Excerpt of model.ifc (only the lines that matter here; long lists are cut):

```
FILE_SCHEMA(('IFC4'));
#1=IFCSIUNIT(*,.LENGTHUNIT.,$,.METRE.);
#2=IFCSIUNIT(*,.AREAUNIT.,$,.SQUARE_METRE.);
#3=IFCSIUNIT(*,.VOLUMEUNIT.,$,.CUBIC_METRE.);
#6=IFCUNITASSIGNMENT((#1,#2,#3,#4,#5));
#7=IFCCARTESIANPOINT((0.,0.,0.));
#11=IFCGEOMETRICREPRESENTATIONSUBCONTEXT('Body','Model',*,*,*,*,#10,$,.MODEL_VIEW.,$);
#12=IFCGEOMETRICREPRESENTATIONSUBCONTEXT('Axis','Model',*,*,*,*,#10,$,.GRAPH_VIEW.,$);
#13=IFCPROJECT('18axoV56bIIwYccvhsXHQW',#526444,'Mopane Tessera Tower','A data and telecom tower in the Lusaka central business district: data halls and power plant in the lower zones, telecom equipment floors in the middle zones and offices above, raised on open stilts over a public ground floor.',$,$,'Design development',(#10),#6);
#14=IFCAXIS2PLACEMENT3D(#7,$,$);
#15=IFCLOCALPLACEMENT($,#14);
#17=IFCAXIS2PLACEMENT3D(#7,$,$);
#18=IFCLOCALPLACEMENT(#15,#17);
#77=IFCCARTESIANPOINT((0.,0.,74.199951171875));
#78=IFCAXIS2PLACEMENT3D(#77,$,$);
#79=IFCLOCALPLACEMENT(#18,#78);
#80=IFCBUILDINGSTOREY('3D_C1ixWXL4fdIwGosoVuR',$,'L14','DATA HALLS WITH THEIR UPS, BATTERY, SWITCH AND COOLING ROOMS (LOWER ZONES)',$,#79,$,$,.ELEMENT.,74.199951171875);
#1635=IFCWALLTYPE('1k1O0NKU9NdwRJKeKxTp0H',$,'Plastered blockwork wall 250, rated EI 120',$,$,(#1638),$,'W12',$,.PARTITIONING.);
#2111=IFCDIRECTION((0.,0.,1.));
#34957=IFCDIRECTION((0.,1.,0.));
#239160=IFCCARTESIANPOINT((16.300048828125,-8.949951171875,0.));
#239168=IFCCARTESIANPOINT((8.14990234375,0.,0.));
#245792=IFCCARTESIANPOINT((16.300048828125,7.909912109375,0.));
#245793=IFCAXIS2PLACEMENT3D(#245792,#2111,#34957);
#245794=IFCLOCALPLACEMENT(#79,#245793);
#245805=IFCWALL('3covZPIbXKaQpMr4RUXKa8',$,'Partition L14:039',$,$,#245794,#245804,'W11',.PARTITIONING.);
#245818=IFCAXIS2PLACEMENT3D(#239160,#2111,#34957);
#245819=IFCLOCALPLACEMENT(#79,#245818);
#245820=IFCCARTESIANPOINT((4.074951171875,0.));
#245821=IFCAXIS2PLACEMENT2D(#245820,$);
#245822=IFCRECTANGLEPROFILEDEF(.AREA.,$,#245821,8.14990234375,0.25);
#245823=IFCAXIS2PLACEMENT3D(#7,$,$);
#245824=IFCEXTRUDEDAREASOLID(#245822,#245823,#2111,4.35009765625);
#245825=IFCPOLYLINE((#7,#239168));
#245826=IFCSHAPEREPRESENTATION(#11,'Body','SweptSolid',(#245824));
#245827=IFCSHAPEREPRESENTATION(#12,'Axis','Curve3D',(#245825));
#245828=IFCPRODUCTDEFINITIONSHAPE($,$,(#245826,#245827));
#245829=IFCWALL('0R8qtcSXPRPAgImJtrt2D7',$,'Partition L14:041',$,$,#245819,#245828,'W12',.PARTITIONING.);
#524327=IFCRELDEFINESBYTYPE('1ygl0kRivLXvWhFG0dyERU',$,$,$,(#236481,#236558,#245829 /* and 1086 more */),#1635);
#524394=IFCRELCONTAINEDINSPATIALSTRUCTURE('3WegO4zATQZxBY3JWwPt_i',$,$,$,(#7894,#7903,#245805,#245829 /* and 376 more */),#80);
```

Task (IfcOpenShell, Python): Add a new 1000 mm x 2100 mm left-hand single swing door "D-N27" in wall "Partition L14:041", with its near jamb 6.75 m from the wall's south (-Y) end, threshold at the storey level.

```python
import numpy as np
import ifcopenshell
import ifcopenshell.api.feature
import ifcopenshell.api.geometry
import ifcopenshell.api.root
import ifcopenshell.api.spatial
import ifcopenshell.geom
import ifcopenshell.util.element
import ifcopenshell.util.placement
import ifcopenshell.util.representation
import ifcopenshell.util.shape
import ifcopenshell.util.unit

model = ifcopenshell.open("model.ifc")
unit_scale = ifcopenshell.util.unit.calculate_unit_scale(model)
settings = ifcopenshell.geom.settings()


def volume(element):
    """Net volume in cubic metres, openings subtracted."""
    shape = ifcopenshell.geom.create_shape(settings, element)
    return ifcopenshell.util.shape.get_volume(shape.geometry)


wall = model.by_guid("0R8qtcSXPRPAgImJtrt2D7")
storey = ifcopenshell.util.element.get_container(wall, ifc_class="IfcBuildingStorey")
context = ifcopenshell.util.representation.get_context(model, "Model", "Body", "MODEL_VIEW")
before = volume(wall)

width, height, from_end, sill = 1, 2.1, 6.75, 0.0  # metres

# The wall runs along its own X axis, and the end named is its -X end.
wall_shape = ifcopenshell.geom.create_shape(settings, wall)
x, y, z = ifcopenshell.util.shape.get_vertices(wall_shape.geometry).T
start = x.min() + from_end
face, thickness = float(y.min()), float(y.max() - y.min())
wall_matrix = ifcopenshell.util.placement.get_local_placement(wall.ObjectPlacement)
level = ifcopenshell.util.placement.get_local_placement(storey.ObjectPlacement)[2, 3]


def in_wall(x, y):
    """Placement at x, y metres in the wall's axes, at sill height."""
    matrix = wall_matrix.copy()
    matrix[:, 3] = wall_matrix @ np.array([x / unit_scale, y / unit_scale, 0.0, 1.0])
    matrix[2, 3] = level + sill / unit_scale
    return matrix


# Opening: a box that overshoots both wall faces by 50 mm.
opening = ifcopenshell.api.root.create_entity(model, ifc_class="IfcOpeningElement", predefined_type="OPENING")
box = ifcopenshell.api.geometry.add_wall_representation(
    model, context=context, length=width, height=height, thickness=thickness + 0.1
)
ifcopenshell.api.geometry.assign_representation(model, product=opening, representation=box)
ifcopenshell.api.geometry.edit_object_placement(model, product=opening, matrix=in_wall(start, face - 0.05), is_si=False)
ifcopenshell.api.feature.add_feature(model, feature=opening, element=wall)

door = ifcopenshell.api.root.create_entity(model, ifc_class="IfcDoor", name="D-N27", predefined_type="DOOR")
door.OverallWidth, door.OverallHeight = width / unit_scale, height / unit_scale
door.OperationType = "SINGLE_SWING_LEFT"
body = ifcopenshell.api.geometry.add_door_representation(
    model,
    context=context,
    overall_width=door.OverallWidth,
    overall_height=door.OverallHeight,
    operation_type="SINGLE_SWING_LEFT",
    lining_properties={"LiningDepth": thickness / unit_scale, "ThresholdDepth": thickness / unit_scale},
)
ifcopenshell.api.geometry.assign_representation(model, product=door, representation=body)
ifcopenshell.api.spatial.assign_container(model, products=[door], relating_structure=storey)
ifcopenshell.api.feature.add_filling(model, opening=opening, element=door)

# The lining spans the wall, so the door starts at the wall face.
ifcopenshell.api.geometry.edit_object_placement(model, product=door, matrix=in_wall(start, face), is_si=False)

after = volume(wall)

print(f"wall volume {before:.3f} -> {after:.3f} m3")

model.write("model-out.ifc")
```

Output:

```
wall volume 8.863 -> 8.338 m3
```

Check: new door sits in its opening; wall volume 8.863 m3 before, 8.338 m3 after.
